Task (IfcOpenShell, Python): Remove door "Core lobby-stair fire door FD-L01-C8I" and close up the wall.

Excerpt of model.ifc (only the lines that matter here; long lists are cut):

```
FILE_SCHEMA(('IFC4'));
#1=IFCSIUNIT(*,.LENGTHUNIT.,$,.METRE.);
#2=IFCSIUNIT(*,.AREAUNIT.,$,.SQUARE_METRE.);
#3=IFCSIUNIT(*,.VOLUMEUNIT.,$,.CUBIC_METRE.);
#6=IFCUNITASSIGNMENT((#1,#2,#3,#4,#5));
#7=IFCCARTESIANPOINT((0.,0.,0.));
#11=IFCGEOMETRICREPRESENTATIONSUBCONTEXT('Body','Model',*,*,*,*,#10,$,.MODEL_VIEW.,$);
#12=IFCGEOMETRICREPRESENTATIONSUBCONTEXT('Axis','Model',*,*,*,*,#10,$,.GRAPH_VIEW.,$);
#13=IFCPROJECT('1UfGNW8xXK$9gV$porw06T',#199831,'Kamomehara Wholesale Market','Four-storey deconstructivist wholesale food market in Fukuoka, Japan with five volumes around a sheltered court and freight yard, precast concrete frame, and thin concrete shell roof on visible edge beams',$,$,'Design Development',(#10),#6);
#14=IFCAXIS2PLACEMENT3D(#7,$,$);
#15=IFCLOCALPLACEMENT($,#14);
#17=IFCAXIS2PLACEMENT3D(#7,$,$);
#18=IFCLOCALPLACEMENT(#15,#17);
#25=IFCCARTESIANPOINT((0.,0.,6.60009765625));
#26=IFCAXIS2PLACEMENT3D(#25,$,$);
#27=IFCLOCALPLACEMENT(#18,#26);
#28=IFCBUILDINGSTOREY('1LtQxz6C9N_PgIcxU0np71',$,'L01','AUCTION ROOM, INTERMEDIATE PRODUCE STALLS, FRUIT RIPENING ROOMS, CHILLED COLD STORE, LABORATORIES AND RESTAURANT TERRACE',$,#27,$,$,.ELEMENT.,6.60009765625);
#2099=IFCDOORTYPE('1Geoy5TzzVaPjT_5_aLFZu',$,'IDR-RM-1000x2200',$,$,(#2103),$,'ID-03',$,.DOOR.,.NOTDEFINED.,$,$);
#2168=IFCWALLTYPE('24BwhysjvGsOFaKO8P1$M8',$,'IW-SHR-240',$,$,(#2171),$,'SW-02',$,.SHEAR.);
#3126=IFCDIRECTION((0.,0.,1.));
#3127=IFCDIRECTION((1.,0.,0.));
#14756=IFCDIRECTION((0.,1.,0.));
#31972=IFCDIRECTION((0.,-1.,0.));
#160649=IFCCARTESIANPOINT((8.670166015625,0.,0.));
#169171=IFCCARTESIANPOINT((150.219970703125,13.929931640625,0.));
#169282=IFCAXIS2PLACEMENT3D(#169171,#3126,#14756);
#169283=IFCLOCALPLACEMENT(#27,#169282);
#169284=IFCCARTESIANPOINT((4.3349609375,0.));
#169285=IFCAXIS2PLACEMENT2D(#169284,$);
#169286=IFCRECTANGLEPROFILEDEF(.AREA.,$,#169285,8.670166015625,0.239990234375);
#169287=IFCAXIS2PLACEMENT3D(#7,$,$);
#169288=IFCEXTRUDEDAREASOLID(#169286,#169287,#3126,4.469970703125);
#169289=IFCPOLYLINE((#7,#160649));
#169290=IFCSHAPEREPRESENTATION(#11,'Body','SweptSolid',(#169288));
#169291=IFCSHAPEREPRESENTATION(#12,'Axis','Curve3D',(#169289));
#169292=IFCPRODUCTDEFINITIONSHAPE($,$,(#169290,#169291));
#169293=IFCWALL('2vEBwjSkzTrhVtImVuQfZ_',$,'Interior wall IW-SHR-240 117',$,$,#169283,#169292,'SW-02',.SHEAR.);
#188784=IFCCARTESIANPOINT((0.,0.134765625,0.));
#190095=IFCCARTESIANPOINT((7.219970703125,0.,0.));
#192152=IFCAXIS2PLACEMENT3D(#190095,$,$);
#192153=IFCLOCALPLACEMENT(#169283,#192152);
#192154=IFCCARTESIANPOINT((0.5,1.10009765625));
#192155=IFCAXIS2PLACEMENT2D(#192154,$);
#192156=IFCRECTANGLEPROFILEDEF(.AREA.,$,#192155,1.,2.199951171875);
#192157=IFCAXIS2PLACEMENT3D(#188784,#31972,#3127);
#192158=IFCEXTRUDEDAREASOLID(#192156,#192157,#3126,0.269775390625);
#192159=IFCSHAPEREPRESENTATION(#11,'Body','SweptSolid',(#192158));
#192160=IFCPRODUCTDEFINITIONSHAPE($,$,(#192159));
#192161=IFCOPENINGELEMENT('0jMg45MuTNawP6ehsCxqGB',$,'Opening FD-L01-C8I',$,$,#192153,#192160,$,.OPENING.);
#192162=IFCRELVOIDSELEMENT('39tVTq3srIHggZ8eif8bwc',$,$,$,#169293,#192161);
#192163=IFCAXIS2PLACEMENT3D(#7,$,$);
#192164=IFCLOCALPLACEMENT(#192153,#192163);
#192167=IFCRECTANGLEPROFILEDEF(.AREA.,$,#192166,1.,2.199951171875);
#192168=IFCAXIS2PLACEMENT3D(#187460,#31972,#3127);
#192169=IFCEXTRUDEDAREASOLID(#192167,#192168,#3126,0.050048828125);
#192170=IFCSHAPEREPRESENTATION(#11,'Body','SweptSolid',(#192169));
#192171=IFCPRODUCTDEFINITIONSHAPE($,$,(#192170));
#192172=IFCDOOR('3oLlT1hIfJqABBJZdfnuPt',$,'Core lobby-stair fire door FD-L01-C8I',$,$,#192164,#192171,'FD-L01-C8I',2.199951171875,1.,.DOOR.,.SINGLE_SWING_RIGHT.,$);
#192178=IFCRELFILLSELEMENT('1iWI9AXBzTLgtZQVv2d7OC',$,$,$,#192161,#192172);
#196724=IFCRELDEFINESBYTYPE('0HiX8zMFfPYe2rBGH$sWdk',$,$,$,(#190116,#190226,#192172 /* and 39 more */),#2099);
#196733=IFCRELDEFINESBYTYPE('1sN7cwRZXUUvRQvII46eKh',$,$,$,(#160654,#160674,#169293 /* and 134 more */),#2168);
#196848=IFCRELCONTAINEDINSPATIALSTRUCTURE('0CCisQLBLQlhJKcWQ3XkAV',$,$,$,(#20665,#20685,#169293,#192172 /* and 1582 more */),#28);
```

```python
import ifcopenshell
import ifcopenshell.api.feature
import ifcopenshell.api.root
import ifcopenshell.geom
import ifcopenshell.util.shape

model = ifcopenshell.open("model.ifc")
settings = ifcopenshell.geom.settings()


def volume(element):
    """Net volume in cubic metres, openings subtracted."""
    shape = ifcopenshell.geom.create_shape(settings, element)
    return ifcopenshell.util.shape.get_volume(shape.geometry)


door = model.by_id(192172)
opening = door.FillsVoids[0].RelatingOpeningElement
wall = opening.VoidsElements[0].RelatingBuildingElement
before = volume(wall)

ifcopenshell.api.root.remove_product(model, product=door)
ifcopenshell.api.feature.remove_feature(model, feature=opening)

after = volume(wall)

print(f"wall volume {before:.3f} -> {after:.3f} m3")

model.write("model_rev.ifc")
```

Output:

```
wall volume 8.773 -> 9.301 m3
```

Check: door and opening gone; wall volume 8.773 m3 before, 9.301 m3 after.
